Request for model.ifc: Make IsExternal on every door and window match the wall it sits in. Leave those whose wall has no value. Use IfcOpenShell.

First a look at what the model holds.

```python
import ifcopenshell
import ifcopenshell.util.element

model = ifcopenshell.open("model.ifc")
print(model.schema)
seen = {}
for e in model.by_type("IfcDoor") + model.by_type("IfcWindow"):
    if not e.FillsVoids:
        continue
    host = e.FillsVoids[0].RelatingOpeningElement.VoidsElements[0].RelatingBuildingElement
    own = ifcopenshell.util.element.get_pset(e, f"Pset_{e.is_a()[3:].removesuffix('StandardCase')}Common", "IsExternal")
    wall = ifcopenshell.util.element.get_pset(host, "Pset_WallCommon", "IsExternal")
    seen[e.is_a(), own, wall] = seen.get((e.is_a(), own, wall), 0) + 1
for (cls, own, wall), count in sorted(seen.items(), key=str):
    print(count, cls, "IsExternal:", own, "| host wall:", wall)
```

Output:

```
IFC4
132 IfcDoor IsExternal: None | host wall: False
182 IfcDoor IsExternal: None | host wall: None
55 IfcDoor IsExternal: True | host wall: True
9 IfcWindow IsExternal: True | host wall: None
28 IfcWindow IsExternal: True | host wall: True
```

```python
import ifcopenshell
import ifcopenshell.api.pset
import ifcopenshell.util.element

model = ifcopenshell.open("model.ifc")

count = 0
for ifc_class, pset_name in (("IfcDoor", "Pset_DoorCommon"), ("IfcWindow", "Pset_WindowCommon")):
    for e in model.by_type(ifc_class):
        if not e.FillsVoids:
            continue
        host = e.FillsVoids[0].RelatingOpeningElement.VoidsElements[0].RelatingBuildingElement
        external = ifcopenshell.util.element.get_pset(host, "Pset_WallCommon", "IsExternal")
        if external is None or ifcopenshell.util.element.get_pset(e, pset_name, "IsExternal") == external:
            continue
        pset = ifcopenshell.api.pset.add_pset(model, product=e, name=pset_name)
        ifcopenshell.api.pset.edit_pset(model, pset=pset, properties={"IsExternal": external})
        count += 1

print(count, "updated")

model.write("model_edited.ifc")
```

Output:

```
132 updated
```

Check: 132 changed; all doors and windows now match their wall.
